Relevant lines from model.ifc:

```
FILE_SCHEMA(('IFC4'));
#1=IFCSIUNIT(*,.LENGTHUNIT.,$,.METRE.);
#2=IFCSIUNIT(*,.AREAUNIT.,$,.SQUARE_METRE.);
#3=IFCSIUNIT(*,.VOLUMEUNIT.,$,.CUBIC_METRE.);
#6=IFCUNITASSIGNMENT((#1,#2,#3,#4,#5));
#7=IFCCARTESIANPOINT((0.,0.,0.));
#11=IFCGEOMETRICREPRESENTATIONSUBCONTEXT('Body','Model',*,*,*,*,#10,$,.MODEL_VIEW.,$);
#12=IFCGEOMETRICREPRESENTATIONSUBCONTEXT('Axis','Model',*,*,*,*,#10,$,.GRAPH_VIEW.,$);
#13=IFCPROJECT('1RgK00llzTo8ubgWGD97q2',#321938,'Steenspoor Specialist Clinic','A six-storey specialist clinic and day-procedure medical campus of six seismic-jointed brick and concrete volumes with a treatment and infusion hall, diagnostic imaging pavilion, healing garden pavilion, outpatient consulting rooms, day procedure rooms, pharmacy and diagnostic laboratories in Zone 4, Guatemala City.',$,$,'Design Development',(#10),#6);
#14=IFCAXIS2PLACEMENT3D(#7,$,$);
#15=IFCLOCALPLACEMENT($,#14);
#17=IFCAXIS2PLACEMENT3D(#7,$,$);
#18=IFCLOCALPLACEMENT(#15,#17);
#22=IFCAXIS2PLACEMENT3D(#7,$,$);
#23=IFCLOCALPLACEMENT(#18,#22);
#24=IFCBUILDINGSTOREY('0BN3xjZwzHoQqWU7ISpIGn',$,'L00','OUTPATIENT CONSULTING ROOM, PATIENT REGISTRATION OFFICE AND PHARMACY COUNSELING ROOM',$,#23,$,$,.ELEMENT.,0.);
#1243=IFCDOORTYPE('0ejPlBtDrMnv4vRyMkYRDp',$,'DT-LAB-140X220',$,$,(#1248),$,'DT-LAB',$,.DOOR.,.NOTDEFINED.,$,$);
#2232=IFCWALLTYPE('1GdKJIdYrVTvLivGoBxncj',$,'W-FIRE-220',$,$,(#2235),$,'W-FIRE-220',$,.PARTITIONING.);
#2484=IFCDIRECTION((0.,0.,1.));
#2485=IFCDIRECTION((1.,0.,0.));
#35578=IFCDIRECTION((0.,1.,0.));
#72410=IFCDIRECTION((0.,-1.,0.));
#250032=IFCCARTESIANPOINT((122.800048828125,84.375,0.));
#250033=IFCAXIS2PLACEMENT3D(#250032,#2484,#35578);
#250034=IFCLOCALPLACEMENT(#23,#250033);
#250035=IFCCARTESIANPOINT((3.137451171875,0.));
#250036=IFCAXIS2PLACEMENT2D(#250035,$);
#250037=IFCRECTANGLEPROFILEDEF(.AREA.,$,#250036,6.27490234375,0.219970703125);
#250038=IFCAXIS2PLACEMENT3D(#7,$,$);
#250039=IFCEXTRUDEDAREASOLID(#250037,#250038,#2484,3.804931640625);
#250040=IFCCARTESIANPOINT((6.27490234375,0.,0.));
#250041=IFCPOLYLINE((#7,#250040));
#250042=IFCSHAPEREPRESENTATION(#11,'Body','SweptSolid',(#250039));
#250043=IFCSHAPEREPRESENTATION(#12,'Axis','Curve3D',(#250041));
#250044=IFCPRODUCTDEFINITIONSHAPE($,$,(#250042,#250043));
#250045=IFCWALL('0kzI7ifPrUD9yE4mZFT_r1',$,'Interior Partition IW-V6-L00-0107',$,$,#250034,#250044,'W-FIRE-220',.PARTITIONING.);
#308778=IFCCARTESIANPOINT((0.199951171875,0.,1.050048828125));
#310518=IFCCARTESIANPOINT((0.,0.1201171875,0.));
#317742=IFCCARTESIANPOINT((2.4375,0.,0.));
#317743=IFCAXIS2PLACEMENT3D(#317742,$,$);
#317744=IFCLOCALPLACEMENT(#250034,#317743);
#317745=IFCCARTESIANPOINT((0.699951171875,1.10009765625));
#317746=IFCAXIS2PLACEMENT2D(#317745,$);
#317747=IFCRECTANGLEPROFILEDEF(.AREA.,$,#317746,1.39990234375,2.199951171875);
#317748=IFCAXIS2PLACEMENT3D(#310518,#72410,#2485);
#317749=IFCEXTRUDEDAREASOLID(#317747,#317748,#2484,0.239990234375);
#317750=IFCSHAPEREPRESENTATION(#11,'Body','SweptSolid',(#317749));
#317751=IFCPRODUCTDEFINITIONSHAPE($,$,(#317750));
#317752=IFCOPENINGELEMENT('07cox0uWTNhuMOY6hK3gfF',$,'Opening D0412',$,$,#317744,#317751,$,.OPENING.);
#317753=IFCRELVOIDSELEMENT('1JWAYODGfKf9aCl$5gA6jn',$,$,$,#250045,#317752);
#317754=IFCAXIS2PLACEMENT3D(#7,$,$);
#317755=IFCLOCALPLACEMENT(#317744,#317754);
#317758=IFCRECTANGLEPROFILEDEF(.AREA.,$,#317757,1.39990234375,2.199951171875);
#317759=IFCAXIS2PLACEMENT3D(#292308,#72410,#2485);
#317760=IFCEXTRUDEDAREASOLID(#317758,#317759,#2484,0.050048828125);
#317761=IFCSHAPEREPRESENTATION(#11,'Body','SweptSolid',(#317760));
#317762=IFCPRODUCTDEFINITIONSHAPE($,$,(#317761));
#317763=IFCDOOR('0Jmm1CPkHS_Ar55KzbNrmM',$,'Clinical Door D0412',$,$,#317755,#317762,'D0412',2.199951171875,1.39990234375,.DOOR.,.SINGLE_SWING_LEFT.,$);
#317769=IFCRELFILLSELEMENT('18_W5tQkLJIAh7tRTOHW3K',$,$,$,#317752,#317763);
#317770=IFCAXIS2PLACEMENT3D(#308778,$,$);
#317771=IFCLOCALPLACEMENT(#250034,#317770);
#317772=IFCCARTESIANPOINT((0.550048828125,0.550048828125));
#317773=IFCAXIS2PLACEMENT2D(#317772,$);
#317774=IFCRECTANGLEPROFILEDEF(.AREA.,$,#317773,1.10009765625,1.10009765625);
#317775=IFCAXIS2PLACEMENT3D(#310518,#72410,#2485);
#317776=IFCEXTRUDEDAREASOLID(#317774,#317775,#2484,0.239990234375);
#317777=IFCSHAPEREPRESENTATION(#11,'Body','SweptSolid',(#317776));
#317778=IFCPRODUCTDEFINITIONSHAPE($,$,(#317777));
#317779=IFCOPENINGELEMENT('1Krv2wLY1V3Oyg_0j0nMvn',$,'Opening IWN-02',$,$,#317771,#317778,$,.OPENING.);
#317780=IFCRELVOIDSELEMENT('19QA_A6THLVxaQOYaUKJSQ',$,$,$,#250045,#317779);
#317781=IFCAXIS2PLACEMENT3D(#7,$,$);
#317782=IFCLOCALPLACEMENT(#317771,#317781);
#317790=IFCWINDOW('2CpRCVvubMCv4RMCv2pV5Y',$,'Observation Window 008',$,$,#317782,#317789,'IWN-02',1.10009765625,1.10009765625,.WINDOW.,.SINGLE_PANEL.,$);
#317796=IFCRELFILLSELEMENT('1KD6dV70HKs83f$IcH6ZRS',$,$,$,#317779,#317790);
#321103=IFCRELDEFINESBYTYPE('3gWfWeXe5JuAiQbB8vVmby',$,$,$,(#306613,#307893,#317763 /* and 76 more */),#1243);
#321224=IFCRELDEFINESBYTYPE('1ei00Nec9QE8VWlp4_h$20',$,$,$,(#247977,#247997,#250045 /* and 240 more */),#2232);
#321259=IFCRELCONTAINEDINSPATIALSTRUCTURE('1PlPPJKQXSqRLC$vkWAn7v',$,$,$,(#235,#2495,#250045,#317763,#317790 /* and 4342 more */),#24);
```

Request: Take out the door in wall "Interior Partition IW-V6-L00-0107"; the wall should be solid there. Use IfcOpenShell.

```python
import ifcopenshell
import ifcopenshell.api.feature
import ifcopenshell.api.root
import ifcopenshell.geom
import ifcopenshell.util.shape

model = ifcopenshell.open("model.ifc")
settings = ifcopenshell.geom.settings()


def volume(element):
    """Net volume in cubic metres, openings subtracted."""
    shape = ifcopenshell.geom.create_shape(settings, element)
    return ifcopenshell.util.shape.get_volume(shape.geometry)


door = model.by_guid("0Jmm1CPkHS_Ar55KzbNrmM")
opening = door.FillsVoids[0].RelatingOpeningElement
wall = opening.VoidsElements[0].RelatingBuildingElement
before = volume(wall)

ifcopenshell.api.root.remove_product(model, product=door)
ifcopenshell.api.feature.remove_feature(model, feature=opening)

after = volume(wall)

print(f"wall volume {before:.3f} -> {after:.3f} m3")

model.write("model_edited.ifc")
```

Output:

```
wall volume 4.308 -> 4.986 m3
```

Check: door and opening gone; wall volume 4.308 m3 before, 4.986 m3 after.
